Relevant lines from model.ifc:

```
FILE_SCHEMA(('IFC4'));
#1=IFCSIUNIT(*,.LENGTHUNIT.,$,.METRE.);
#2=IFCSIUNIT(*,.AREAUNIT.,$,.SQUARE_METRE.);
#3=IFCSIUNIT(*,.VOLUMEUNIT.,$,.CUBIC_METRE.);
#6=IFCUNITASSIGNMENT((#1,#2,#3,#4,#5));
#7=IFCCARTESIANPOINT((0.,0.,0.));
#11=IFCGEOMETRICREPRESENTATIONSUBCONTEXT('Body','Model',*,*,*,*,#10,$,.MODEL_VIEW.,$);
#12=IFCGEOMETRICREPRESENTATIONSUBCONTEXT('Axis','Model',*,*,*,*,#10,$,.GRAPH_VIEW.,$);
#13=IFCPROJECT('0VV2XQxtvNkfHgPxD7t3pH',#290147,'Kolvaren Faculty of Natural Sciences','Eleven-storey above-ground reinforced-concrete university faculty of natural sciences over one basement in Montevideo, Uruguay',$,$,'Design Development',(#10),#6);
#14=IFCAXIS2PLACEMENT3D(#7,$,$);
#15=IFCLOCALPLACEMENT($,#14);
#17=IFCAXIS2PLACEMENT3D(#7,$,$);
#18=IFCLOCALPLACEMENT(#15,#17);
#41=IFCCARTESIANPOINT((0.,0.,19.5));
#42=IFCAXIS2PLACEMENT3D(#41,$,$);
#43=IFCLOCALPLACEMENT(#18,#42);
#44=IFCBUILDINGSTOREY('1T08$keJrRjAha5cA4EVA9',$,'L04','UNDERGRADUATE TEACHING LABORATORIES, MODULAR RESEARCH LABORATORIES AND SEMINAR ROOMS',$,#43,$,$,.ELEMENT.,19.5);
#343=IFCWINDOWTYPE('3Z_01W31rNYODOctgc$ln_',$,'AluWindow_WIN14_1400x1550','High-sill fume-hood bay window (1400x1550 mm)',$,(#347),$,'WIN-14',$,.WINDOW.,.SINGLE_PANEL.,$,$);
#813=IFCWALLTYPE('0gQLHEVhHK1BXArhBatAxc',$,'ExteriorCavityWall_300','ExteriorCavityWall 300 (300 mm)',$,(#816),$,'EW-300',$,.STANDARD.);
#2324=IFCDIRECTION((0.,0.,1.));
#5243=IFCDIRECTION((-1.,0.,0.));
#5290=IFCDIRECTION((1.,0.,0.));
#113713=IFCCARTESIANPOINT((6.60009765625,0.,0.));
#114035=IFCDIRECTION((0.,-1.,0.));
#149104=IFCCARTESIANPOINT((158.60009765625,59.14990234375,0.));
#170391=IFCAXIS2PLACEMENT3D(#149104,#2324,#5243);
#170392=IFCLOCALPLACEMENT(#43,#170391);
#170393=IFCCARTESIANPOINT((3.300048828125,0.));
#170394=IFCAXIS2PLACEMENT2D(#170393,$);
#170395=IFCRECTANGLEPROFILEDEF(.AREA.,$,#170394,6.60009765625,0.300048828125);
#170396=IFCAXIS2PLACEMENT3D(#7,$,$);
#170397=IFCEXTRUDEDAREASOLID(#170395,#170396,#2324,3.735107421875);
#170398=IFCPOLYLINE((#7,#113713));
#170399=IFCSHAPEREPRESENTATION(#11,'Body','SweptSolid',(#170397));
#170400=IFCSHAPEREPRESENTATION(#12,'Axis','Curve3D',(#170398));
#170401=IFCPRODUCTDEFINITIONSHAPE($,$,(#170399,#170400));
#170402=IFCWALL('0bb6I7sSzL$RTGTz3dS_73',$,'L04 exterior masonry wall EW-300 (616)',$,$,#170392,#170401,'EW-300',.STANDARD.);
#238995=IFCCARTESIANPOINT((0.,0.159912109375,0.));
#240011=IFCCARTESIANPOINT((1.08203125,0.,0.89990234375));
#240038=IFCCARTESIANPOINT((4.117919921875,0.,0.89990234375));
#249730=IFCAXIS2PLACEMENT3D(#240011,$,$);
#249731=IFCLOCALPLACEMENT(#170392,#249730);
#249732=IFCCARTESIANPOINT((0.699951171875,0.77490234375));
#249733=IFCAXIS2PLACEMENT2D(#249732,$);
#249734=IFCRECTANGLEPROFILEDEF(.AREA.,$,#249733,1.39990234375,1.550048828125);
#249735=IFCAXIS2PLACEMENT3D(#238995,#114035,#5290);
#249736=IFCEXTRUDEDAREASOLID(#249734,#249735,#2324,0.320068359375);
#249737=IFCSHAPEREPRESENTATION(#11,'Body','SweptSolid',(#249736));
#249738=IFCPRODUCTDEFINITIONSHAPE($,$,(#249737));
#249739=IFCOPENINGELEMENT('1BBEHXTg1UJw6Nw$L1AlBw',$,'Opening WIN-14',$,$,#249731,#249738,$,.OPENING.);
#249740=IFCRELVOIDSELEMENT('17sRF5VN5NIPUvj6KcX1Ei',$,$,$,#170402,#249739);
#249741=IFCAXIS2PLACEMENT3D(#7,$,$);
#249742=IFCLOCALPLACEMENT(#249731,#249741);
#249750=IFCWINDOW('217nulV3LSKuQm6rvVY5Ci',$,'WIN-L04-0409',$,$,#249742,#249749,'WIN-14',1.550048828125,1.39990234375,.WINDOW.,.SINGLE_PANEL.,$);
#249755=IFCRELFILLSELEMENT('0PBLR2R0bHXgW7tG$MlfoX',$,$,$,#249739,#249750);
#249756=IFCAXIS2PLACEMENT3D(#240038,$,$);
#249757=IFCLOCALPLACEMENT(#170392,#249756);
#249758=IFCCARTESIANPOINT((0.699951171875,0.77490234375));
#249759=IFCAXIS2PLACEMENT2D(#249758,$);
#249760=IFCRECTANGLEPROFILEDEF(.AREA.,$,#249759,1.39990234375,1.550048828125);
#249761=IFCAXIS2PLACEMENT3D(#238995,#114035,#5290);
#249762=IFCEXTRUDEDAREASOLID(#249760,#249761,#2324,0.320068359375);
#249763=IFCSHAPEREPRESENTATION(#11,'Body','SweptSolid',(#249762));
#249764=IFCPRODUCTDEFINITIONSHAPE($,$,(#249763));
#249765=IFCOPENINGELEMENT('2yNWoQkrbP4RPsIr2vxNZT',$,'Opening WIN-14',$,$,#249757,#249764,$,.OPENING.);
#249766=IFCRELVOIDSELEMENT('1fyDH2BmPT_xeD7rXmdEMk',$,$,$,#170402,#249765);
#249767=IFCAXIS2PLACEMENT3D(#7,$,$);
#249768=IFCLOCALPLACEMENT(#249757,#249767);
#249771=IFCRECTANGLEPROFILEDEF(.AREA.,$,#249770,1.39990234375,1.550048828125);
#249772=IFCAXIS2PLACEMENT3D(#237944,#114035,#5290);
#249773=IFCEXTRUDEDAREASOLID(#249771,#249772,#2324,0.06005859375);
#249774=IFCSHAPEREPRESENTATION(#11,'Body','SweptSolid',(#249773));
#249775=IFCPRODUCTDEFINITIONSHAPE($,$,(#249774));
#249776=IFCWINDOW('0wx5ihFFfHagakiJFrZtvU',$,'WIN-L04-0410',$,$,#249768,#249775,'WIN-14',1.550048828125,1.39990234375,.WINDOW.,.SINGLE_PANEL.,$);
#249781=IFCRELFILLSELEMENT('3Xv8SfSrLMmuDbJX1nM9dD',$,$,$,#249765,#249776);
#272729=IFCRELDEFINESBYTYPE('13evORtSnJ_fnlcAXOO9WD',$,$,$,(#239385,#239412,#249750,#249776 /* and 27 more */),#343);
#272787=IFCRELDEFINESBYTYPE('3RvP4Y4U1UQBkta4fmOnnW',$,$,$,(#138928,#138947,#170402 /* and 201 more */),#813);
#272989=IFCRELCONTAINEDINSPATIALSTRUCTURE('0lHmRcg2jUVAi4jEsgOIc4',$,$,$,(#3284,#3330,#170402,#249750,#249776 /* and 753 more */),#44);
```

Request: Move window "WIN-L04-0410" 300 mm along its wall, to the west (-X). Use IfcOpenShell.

```python
import ifcopenshell
import ifcopenshell.api.geometry
import ifcopenshell.util.placement
import ifcopenshell.util.unit

model = ifcopenshell.open("model.ifc")
unit_scale = ifcopenshell.util.unit.calculate_unit_scale(model)

window = model.by_guid("0wx5ihFFfHagakiJFrZtvU")
opening = window.FillsVoids[0].RelatingOpeningElement
wall = opening.VoidsElements[0].RelatingBuildingElement

wall_matrix = ifcopenshell.util.placement.get_local_placement(wall.ObjectPlacement)
shift = wall_matrix[:3, 0] * 0.3 / unit_scale
before = ifcopenshell.util.placement.get_local_placement(window.ObjectPlacement)[:3, 3].copy()

# The window is placed relative to its opening, so it follows when the opening moves.
matrix = ifcopenshell.util.placement.get_local_placement(opening.ObjectPlacement)
matrix[:3, 3] += shift
ifcopenshell.api.geometry.edit_object_placement(
    model, product=opening, matrix=matrix, is_si=False, should_transform_children=True
)

after = ifcopenshell.util.placement.get_local_placement(window.ObjectPlacement)[:3, 3]
print("window moved by", (after - before).round(3) + 0.0)

model.write("model_edited.ifc")
```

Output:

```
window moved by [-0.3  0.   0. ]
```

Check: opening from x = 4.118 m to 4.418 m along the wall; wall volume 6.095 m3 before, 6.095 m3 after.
